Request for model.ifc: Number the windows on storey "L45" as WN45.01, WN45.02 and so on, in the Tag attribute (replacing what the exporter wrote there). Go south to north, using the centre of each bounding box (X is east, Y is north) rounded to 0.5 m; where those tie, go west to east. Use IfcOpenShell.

First a look at what the model holds.

```python
import ifcopenshell
import ifcopenshell.util.element
import ifcopenshell.util.placement

model = ifcopenshell.open("model.ifc")
print(model.schema)
storey = next(s for s in model.by_type("IfcBuildingStorey") if s.Name == "L45")
windows = [e for e in ifcopenshell.util.element.get_decomposition(storey) if e.is_a("IfcWindow")]
for e in sorted(windows, key=lambda e: e.id()):
    origin = ifcopenshell.util.placement.get_local_placement(e.ObjectPlacement)[:3, 3]
    print(e.id(), e.Tag, e.Name, origin.round(2) + 0.0, sep=" | ")
```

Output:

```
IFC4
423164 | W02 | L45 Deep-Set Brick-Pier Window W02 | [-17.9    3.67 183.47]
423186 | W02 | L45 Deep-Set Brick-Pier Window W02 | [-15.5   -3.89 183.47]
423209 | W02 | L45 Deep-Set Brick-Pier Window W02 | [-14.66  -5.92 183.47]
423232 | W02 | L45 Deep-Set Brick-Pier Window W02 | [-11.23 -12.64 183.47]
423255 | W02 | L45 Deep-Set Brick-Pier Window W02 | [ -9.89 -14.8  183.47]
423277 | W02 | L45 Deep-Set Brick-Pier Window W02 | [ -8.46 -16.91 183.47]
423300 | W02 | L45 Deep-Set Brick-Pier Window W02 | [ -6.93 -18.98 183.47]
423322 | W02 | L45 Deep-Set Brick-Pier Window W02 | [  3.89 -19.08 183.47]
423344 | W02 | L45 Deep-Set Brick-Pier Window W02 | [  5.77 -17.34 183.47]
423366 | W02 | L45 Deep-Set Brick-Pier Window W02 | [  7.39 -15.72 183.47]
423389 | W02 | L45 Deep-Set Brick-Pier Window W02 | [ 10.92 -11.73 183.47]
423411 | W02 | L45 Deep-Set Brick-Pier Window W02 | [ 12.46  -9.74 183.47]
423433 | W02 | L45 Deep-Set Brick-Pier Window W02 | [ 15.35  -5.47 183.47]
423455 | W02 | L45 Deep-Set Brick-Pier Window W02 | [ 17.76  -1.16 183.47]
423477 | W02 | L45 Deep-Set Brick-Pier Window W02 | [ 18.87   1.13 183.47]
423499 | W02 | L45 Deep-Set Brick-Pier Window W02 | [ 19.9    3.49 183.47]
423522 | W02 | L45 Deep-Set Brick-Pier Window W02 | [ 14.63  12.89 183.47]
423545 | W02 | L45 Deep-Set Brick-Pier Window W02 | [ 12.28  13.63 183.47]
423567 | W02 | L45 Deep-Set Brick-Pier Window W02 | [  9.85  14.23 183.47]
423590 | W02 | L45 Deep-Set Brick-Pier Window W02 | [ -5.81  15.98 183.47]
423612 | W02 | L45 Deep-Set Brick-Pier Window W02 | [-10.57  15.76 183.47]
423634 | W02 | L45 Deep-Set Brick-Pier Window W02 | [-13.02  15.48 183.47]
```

```python
import ifcopenshell
import ifcopenshell.geom
import ifcopenshell.util.element
import ifcopenshell.util.shape

model = ifcopenshell.open("model.ifc")
settings = ifcopenshell.geom.settings()
settings.set("use-world-coords", True)


def centre(element):
    shape = ifcopenshell.geom.create_shape(settings, element)
    return ifcopenshell.util.shape.get_bbox_centroid(shape.geometry)


storey = next(s for s in model.by_type("IfcBuildingStorey") if s.Name == "L45")
windows = [e for e in ifcopenshell.util.element.get_decomposition(storey) if e.is_a("IfcWindow")]

# Insertion points can sit at a corner or the storey origin, so sort by the geometry (in metres).
centres = {e: centre(e) for e in windows}
windows.sort(key=lambda e: (round(centres[e][1] / 0.5), centres[e][0]))

for i, e in enumerate(windows, start=1):
    number = f"WN45.{i:02d}"
    e.Tag = number
    print(e.id(), number)

model.write("model_v2.ifc")
```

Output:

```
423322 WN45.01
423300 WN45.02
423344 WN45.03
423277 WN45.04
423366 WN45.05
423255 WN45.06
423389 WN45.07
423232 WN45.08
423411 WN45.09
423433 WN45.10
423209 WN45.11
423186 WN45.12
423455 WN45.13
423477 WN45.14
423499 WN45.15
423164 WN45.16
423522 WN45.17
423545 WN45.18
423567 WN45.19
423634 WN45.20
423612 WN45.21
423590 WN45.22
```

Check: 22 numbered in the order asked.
